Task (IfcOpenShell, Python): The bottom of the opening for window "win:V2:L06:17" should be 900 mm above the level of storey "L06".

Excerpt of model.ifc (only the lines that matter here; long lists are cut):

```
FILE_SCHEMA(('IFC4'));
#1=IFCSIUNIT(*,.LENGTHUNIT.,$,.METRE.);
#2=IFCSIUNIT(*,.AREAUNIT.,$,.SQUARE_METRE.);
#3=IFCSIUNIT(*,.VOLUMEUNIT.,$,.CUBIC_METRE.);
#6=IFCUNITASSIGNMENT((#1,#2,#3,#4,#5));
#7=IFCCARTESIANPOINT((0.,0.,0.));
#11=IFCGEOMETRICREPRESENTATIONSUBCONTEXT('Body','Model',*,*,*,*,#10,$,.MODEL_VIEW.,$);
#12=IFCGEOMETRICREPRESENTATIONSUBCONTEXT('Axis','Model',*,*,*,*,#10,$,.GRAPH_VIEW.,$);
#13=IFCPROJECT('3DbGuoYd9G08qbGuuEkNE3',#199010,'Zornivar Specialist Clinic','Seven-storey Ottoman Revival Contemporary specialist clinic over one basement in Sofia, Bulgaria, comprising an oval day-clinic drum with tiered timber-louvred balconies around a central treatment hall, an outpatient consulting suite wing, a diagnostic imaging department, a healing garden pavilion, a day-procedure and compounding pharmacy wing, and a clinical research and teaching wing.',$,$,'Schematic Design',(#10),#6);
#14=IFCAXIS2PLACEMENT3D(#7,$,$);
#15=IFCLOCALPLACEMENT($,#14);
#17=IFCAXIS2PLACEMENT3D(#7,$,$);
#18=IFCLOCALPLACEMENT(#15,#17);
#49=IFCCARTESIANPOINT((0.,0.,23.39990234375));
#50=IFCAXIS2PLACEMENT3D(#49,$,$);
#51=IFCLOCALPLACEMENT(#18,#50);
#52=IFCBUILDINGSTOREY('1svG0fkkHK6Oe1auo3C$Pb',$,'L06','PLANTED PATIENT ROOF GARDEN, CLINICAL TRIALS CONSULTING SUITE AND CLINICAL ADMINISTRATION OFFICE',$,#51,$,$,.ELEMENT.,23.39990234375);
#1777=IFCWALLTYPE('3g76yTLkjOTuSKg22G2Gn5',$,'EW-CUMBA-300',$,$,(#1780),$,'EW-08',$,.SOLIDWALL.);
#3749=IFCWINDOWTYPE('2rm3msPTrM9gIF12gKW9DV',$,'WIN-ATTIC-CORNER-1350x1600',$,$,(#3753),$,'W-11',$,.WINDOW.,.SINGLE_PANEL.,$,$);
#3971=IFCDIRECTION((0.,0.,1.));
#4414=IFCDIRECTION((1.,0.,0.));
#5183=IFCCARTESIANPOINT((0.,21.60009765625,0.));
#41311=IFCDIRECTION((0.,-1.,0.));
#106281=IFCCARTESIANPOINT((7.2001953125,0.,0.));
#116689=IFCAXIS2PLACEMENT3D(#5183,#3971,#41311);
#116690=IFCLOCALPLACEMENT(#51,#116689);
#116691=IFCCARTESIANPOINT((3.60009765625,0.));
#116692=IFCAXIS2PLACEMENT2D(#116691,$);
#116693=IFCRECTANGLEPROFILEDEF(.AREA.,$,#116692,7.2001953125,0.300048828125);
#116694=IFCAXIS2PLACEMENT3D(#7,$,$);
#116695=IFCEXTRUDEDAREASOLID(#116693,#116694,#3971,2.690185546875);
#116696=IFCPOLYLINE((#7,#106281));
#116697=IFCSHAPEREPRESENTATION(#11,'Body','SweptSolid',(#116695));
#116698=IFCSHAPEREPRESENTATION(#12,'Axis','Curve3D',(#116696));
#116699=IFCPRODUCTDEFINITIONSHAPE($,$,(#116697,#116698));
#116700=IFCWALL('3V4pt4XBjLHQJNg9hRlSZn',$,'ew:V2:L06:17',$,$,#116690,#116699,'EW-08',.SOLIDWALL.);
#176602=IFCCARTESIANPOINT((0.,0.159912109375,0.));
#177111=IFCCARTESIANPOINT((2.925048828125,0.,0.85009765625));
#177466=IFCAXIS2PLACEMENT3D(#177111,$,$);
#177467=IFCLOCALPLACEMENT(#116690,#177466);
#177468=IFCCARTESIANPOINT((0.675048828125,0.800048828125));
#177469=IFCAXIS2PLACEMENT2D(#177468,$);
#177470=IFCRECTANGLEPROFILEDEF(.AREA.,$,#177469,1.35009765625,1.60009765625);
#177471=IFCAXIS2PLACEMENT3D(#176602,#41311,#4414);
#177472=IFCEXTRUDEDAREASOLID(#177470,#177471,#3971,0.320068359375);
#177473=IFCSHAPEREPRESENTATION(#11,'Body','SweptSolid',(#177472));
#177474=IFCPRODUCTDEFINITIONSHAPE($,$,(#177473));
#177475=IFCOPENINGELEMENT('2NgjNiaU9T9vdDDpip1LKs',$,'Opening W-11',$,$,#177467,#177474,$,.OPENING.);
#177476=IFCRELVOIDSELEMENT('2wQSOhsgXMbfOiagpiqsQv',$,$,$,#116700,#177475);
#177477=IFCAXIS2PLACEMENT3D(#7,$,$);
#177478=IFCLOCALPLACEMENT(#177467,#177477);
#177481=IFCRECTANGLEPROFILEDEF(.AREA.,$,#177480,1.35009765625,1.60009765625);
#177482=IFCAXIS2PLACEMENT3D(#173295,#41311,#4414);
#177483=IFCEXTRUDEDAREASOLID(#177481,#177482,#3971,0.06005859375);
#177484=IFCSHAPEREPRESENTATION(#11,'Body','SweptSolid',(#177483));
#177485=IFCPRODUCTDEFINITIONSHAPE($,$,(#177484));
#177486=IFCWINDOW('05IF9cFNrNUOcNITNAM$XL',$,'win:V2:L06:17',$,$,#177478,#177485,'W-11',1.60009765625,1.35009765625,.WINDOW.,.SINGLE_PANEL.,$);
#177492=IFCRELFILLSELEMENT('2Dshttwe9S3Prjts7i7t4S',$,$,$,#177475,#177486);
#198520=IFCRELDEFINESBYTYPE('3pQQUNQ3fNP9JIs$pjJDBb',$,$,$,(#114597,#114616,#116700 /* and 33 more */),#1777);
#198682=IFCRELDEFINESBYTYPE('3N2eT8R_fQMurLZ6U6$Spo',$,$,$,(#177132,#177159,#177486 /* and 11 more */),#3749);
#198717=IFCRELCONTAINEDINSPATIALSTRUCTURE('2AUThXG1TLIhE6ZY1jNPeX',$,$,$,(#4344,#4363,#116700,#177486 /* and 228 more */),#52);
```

```python
import numpy as np
import ifcopenshell
import ifcopenshell.api.geometry
import ifcopenshell.geom
import ifcopenshell.util.element
import ifcopenshell.util.placement
import ifcopenshell.util.shape
import ifcopenshell.util.unit

model = ifcopenshell.open("model.ifc")
unit_scale = ifcopenshell.util.unit.calculate_unit_scale(model)

window = model.by_guid("05IF9cFNrNUOcNITNAM$XL")
opening = window.FillsVoids[0].RelatingOpeningElement
storey = ifcopenshell.util.element.get_container(window, ifc_class="IfcBuildingStorey")
level = ifcopenshell.util.placement.get_local_placement(storey.ObjectPlacement)[2, 3]

# The opening's origin need not be at the sill, so measure its lowest point.
shape = ifcopenshell.geom.create_shape(ifcopenshell.geom.settings(), opening)
bottom = ifcopenshell.util.shape.get_shape_bottom_elevation(shape, shape.geometry) / unit_scale
dz = level + 0.9 - bottom

shift = np.array([0.0, 0.0, dz])
# The window is placed relative to its opening, so it follows when the opening moves.
matrix = ifcopenshell.util.placement.get_local_placement(opening.ObjectPlacement)
matrix[:3, 3] += shift
ifcopenshell.api.geometry.edit_object_placement(
    model, product=opening, matrix=matrix, is_si=False, should_transform_children=True
)

print(f"moved by {dz * unit_scale:+.3f} m")

model.write("model-out.ifc")
```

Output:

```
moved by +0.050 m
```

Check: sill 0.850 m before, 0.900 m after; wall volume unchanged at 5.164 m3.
